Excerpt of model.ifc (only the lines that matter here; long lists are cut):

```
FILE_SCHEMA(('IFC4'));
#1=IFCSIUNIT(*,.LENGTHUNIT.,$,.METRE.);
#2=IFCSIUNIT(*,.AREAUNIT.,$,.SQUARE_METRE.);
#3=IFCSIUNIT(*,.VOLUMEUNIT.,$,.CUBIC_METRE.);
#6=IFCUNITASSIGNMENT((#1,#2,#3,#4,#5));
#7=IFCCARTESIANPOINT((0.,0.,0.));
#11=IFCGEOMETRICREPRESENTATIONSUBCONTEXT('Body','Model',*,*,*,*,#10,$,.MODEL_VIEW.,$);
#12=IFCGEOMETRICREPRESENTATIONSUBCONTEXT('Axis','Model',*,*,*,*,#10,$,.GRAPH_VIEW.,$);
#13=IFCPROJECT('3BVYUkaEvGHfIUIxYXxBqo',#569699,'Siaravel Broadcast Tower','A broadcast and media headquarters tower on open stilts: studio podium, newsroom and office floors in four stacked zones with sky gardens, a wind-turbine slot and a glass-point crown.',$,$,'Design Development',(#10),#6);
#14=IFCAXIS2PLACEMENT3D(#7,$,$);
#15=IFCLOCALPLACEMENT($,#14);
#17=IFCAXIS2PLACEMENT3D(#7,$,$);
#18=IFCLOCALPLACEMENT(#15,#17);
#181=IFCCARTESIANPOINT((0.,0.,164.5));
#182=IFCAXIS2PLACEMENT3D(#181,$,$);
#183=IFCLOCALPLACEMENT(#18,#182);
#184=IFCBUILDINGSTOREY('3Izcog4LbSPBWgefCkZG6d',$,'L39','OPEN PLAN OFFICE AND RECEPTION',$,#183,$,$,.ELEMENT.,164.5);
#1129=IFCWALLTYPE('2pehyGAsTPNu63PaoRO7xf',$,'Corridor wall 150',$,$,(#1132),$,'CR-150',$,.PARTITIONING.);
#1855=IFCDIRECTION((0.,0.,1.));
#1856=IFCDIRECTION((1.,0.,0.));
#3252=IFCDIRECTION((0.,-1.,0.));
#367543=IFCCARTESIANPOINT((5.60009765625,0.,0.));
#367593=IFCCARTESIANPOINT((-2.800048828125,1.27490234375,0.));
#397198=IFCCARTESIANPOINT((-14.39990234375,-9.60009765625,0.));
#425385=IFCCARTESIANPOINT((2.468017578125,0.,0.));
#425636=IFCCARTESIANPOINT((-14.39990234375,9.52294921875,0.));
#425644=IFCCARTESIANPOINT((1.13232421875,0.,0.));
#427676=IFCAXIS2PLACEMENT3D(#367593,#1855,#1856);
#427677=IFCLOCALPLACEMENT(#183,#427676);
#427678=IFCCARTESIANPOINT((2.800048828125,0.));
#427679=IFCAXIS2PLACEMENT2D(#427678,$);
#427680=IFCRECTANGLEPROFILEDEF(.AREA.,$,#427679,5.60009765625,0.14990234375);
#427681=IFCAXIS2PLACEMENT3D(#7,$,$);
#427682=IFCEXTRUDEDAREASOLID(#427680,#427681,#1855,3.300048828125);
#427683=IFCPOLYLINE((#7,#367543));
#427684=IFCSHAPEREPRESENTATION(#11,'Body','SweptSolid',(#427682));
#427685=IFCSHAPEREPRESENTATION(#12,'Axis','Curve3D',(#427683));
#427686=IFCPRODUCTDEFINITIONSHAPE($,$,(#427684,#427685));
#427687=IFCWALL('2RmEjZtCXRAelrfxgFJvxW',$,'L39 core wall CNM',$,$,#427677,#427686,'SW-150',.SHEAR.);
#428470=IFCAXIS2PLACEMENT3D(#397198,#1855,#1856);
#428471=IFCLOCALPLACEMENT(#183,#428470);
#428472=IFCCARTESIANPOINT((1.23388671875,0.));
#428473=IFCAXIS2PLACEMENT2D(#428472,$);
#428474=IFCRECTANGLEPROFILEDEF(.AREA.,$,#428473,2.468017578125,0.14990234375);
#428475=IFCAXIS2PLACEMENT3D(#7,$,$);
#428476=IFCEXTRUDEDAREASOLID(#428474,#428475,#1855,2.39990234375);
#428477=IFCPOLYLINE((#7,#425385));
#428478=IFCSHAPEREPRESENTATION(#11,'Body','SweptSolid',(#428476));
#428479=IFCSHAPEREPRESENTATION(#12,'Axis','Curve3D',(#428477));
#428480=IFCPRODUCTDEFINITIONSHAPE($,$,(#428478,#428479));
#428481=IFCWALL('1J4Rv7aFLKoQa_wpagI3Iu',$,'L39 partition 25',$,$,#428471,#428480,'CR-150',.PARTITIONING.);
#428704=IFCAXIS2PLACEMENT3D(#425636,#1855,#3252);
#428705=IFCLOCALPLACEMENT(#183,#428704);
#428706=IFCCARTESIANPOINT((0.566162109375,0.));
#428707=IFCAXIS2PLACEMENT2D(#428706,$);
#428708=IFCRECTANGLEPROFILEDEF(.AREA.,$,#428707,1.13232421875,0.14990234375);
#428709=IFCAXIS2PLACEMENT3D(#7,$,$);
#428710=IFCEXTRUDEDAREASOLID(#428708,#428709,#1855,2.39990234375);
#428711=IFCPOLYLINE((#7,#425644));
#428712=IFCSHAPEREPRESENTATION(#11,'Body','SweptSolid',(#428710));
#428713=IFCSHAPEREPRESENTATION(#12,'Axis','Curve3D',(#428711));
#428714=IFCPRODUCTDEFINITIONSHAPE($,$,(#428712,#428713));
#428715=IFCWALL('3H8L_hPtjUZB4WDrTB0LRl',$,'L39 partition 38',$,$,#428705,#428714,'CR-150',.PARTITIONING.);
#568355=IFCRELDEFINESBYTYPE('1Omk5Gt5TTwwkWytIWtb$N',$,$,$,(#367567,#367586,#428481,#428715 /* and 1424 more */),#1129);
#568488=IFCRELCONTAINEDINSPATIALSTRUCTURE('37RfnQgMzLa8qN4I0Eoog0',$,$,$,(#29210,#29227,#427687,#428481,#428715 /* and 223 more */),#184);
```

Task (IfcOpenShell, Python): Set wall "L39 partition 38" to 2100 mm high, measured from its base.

```python
import ifcopenshell
import ifcopenshell.geom
import ifcopenshell.util.representation
import ifcopenshell.util.shape
import ifcopenshell.util.unit

model = ifcopenshell.open("model.ifc")
unit_scale = ifcopenshell.util.unit.calculate_unit_scale(model)
settings = ifcopenshell.geom.settings()


def volume(element):
    """Net volume in cubic metres, openings subtracted."""
    shape = ifcopenshell.geom.create_shape(settings, element)
    return ifcopenshell.util.shape.get_volume(shape.geometry)


wall = model.by_guid("3H8L_hPtjUZB4WDrTB0LRl")
before = volume(wall)

body = ifcopenshell.util.representation.get_representation(wall, "Model", "Body")
solid = body.Items[0]
old_height = solid.Depth
solid.Depth = 2.1 / unit_scale
after = volume(wall)

print(f"height {old_height:g} -> {solid.Depth:g}, volume {before:.3f} -> {after:.3f} m3")

model.write("model_edited.ifc")
```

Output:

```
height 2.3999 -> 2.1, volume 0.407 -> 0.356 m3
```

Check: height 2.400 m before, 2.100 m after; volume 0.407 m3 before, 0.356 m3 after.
